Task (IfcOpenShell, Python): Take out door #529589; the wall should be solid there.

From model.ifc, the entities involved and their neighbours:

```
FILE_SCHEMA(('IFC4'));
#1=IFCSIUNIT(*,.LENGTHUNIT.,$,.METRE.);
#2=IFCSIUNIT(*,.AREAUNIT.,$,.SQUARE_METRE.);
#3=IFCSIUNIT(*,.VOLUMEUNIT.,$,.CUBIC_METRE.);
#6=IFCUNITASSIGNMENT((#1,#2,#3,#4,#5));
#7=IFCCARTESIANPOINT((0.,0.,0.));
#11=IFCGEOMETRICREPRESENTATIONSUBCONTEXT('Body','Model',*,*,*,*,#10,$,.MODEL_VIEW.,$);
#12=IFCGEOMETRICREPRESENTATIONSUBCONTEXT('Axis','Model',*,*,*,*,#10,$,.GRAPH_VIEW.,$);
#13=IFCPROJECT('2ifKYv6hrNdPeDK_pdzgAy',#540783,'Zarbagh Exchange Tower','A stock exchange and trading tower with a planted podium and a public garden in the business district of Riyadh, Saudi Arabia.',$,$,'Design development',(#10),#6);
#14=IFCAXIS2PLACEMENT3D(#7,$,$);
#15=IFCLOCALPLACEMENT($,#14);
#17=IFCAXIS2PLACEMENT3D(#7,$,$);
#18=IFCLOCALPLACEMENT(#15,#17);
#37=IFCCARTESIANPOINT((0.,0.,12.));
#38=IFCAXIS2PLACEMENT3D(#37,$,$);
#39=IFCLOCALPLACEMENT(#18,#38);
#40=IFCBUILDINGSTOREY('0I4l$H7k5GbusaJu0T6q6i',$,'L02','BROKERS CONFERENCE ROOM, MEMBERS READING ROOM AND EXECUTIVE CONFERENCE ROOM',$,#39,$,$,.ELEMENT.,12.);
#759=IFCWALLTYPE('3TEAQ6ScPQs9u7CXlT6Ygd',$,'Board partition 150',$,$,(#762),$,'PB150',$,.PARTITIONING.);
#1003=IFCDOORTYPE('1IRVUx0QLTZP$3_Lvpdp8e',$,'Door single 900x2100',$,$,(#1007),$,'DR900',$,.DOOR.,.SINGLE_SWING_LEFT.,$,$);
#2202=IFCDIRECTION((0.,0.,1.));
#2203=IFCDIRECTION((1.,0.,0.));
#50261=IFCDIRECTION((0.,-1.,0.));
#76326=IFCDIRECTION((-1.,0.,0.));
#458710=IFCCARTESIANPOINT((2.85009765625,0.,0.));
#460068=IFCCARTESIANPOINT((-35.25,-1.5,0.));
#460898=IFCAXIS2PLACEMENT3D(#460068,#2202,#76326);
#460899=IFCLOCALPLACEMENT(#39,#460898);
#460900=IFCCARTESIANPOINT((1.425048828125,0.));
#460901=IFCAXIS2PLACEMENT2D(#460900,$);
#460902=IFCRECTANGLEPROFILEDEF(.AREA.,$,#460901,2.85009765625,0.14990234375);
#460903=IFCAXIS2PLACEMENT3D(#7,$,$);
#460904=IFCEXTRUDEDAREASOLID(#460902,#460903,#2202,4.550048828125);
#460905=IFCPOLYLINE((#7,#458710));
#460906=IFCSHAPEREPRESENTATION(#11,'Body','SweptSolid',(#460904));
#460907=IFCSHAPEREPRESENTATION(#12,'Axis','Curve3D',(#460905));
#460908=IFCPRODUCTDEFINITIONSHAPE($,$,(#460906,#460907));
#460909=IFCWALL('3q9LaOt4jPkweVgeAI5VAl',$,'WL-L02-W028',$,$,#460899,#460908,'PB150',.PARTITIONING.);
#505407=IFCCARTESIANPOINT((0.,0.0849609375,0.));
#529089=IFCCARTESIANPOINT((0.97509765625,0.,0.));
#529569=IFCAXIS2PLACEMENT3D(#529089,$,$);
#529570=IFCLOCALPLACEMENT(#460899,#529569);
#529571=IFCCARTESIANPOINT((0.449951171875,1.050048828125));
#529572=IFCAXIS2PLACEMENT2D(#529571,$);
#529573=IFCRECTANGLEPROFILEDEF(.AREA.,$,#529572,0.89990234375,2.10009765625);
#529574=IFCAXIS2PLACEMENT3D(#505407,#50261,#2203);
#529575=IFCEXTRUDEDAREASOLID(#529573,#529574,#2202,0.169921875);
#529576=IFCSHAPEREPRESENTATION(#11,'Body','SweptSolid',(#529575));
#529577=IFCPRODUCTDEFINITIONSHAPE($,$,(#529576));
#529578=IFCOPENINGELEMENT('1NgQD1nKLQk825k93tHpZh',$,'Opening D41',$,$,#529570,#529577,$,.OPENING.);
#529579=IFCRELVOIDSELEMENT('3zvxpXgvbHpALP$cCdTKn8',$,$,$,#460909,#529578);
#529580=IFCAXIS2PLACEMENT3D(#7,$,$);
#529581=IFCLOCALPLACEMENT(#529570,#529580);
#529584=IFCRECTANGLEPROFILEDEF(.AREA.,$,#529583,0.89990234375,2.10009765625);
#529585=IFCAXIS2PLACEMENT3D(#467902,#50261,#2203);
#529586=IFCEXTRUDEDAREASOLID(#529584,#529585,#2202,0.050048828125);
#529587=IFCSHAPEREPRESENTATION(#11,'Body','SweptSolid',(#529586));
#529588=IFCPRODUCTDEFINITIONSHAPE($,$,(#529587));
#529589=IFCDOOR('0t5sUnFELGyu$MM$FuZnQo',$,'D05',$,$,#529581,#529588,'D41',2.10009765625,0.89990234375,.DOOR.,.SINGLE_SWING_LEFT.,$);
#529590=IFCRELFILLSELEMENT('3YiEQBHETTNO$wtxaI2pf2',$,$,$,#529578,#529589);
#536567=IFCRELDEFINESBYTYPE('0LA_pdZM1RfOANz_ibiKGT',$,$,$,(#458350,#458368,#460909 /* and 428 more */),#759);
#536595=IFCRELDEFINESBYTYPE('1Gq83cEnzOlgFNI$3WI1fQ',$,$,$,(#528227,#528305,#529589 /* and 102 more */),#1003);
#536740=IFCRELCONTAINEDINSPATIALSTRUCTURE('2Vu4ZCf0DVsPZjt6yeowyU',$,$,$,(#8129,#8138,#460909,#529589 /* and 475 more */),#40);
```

```python
import ifcopenshell
import ifcopenshell.api.feature
import ifcopenshell.api.root
import ifcopenshell.geom
import ifcopenshell.util.shape

model = ifcopenshell.open("model.ifc")
settings = ifcopenshell.geom.settings()


def volume(element):
    """Net volume in cubic metres, openings subtracted."""
    shape = ifcopenshell.geom.create_shape(settings, element)
    return ifcopenshell.util.shape.get_volume(shape.geometry)


door = model.by_guid("0t5sUnFELGyu$MM$FuZnQo")
opening = door.FillsVoids[0].RelatingOpeningElement
wall = opening.VoidsElements[0].RelatingBuildingElement
before = volume(wall)

ifcopenshell.api.root.remove_product(model, product=door)
ifcopenshell.api.feature.remove_feature(model, feature=opening)

after = volume(wall)

print(f"wall volume {before:.3f} -> {after:.3f} m3")

model.write("model_edited.ifc")
```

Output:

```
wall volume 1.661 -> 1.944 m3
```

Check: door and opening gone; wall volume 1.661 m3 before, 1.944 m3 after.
